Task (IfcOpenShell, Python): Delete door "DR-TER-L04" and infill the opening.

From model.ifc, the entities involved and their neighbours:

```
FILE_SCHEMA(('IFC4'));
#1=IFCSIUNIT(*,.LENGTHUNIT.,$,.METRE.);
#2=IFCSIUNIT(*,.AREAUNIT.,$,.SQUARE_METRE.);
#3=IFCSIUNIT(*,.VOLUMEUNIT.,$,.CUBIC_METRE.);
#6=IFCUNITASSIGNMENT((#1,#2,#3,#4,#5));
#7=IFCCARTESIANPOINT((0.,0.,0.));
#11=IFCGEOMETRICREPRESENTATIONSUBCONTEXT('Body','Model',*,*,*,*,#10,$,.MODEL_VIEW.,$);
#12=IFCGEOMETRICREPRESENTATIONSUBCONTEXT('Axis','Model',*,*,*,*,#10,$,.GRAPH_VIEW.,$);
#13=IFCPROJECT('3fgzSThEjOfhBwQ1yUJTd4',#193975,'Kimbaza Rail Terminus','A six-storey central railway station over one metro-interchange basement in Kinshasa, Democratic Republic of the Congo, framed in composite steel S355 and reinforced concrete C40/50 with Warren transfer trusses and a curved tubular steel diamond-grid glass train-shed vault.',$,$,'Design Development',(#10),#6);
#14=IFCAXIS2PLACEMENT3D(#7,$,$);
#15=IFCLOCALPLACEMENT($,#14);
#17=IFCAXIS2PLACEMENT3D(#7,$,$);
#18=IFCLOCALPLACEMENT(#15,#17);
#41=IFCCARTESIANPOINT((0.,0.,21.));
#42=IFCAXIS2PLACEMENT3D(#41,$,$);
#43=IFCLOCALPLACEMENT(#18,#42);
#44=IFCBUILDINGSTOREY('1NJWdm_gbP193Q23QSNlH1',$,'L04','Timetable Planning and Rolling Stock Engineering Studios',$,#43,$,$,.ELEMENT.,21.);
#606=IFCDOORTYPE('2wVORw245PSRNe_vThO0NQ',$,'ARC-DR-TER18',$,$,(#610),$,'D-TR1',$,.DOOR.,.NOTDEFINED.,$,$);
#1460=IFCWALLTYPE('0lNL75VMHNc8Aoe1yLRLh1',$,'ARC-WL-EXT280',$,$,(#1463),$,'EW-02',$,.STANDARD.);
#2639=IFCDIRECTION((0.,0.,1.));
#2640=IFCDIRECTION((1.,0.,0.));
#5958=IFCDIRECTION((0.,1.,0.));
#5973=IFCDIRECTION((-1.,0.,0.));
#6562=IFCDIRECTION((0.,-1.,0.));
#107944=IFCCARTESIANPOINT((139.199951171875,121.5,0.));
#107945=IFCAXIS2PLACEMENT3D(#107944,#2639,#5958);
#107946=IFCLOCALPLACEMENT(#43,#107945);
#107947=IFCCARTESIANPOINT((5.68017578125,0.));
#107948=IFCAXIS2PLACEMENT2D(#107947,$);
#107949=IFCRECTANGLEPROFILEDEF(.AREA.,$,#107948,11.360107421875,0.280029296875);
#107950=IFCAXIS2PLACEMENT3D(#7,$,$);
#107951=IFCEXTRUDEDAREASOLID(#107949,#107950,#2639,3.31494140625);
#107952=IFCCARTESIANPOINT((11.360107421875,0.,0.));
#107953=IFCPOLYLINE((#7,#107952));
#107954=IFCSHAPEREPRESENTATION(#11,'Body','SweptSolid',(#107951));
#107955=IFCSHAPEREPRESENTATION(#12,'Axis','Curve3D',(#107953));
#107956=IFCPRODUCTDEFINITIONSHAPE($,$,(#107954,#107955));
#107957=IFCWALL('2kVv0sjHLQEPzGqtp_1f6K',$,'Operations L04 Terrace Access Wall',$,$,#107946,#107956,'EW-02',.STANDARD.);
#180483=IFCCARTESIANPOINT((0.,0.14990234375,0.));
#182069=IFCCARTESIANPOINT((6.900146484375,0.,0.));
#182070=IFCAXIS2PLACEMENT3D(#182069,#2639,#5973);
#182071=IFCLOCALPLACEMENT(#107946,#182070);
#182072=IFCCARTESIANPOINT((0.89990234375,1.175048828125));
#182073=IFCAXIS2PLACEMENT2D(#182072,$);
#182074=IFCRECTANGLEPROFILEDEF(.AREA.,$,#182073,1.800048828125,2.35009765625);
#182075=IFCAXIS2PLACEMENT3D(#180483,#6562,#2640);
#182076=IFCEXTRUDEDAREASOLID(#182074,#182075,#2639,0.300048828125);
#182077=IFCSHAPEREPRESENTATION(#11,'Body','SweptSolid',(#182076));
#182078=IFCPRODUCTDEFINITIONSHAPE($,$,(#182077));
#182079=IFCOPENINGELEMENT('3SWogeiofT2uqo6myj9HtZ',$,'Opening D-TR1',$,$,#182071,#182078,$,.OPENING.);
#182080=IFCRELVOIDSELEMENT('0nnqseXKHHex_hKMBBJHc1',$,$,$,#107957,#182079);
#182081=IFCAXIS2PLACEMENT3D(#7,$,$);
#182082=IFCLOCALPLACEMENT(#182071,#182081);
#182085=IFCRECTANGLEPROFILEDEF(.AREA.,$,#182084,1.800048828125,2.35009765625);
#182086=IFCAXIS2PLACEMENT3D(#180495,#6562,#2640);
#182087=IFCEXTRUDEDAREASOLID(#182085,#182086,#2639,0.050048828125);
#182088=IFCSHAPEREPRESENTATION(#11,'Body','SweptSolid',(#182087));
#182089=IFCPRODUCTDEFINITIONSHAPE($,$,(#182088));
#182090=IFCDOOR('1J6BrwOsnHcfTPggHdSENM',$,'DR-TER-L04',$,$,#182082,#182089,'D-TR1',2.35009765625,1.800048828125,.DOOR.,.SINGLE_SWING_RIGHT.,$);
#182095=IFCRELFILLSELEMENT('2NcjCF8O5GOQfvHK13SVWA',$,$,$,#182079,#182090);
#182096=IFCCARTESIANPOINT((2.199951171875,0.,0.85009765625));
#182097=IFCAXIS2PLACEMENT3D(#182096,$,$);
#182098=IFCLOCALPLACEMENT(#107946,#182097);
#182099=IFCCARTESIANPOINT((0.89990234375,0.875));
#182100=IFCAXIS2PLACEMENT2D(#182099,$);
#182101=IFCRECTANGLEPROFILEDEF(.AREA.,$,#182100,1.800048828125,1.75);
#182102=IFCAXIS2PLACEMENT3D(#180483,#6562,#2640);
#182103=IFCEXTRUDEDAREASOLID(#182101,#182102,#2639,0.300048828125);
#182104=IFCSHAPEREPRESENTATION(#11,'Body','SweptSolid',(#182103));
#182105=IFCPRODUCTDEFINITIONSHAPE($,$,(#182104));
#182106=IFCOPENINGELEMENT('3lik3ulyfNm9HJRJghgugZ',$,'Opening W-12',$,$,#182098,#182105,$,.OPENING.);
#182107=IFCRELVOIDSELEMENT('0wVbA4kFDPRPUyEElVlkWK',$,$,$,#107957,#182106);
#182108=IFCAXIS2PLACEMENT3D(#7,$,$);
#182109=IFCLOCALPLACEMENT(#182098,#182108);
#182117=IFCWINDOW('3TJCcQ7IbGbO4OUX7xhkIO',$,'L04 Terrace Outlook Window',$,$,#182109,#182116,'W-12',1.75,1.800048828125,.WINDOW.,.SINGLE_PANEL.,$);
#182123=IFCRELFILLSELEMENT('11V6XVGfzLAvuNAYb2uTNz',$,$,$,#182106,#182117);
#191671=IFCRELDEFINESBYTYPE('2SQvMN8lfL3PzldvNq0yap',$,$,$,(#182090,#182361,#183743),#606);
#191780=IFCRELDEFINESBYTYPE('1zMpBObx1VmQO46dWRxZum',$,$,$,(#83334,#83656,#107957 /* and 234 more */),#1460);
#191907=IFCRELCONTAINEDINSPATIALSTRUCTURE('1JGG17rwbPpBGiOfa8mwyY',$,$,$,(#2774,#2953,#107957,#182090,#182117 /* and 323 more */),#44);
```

```python
import ifcopenshell
import ifcopenshell.api.feature
import ifcopenshell.api.root
import ifcopenshell.geom
import ifcopenshell.util.shape

model = ifcopenshell.open("model.ifc")
settings = ifcopenshell.geom.settings()


def volume(element):
    """Net volume in cubic metres, openings subtracted."""
    shape = ifcopenshell.geom.create_shape(settings, element)
    return ifcopenshell.util.shape.get_volume(shape.geometry)


door = model.by_guid("1J6BrwOsnHcfTPggHdSENM")
opening = door.FillsVoids[0].RelatingOpeningElement
wall = opening.VoidsElements[0].RelatingBuildingElement
before = volume(wall)

ifcopenshell.api.root.remove_product(model, product=door)
ifcopenshell.api.feature.remove_feature(model, feature=opening)

after = volume(wall)

print(f"wall volume {before:.3f} -> {after:.3f} m3")

model.write("model_edited.ifc")
```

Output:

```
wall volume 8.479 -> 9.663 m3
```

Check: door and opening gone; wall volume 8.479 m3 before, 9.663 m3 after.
